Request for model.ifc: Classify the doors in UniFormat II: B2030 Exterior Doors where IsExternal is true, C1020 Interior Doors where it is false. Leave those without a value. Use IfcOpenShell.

First a look at what the model holds.

```python
import ifcopenshell
import ifcopenshell.util.element

model = ifcopenshell.open("model.ifc")
print(model.schema)
print("classifications:", [c.Name for c in model.by_type("IfcClassification")])
values = [ifcopenshell.util.element.get_pset(e, "Pset_DoorCommon", "IsExternal") for e in model.by_type("IfcDoor")]
for value in (True, False, None):
    print("IsExternal", value, values.count(value))
```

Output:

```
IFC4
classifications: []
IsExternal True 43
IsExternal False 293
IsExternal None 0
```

```python
import ifcopenshell
import ifcopenshell.api.classification
import ifcopenshell.util.element

model = ifcopenshell.open("model.ifc")

system = ifcopenshell.api.classification.add_classification(model, classification="UniFormat II")

doors = model.by_type("IfcDoor")
external = {e: ifcopenshell.util.element.get_pset(e, "Pset_DoorCommon", "IsExternal") for e in doors}
for flag, code, name in ((True, "B2030", "Exterior Doors"), (False, "C1020", "Interior Doors")):
    products = [e for e in doors if external[e] is flag]
    ifcopenshell.api.classification.add_reference(
        model, products=products, classification=system, identification=code, name=name
    )
    print(code, len(products))

model.write("model_edited.ifc")
```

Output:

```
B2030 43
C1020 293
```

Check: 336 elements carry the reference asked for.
